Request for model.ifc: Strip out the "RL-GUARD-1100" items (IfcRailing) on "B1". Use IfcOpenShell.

First a look at what the model holds.

```python
import ifcopenshell
import ifcopenshell.util.element

model = ifcopenshell.open("model.ifc")
print(model.schema)
storey = next(s for s in model.by_type("IfcBuildingStorey") if s.Name == "B1")
railings = [e for e in ifcopenshell.util.element.get_decomposition(storey) if e.is_a("IfcRailing")]
seen = {}
for e in railings:
    element_type = ifcopenshell.util.element.get_type(e)
    name = element_type.Name if element_type not in (None, e) else None
    seen[name] = seen.get(name, 0) + 1
for name, count in sorted(seen.items(), key=str):
    print(count, "x", name)
```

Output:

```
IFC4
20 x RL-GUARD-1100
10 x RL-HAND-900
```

```python
import ifcopenshell
import ifcopenshell.api.root
import ifcopenshell.util.element

model = ifcopenshell.open("model.ifc")

storey = next(s for s in model.by_type("IfcBuildingStorey") if s.Name == "B1")
railings = [e for e in ifcopenshell.util.element.get_decomposition(storey) if e.is_a("IfcRailing")]
targets = [e for e in railings if (t := ifcopenshell.util.element.get_type(e)) not in (None, e) and t.Name == "RL-GUARD-1100"]

for e in targets:
    ifcopenshell.api.root.remove_product(model, product=e)
print(len(targets), "removed")

model.write("model-out.ifc")
```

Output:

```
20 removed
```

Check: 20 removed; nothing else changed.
